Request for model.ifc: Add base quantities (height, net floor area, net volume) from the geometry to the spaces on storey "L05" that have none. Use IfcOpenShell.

First a look at what the model holds.

```python
import ifcopenshell
import ifcopenshell.util.element
import ifcopenshell.util.unit

model = ifcopenshell.open("model.ifc")
print(model.schema)
for unit_type in ("LENGTHUNIT", "AREAUNIT", "VOLUMEUNIT"):
    print(unit_type, ifcopenshell.util.unit.calculate_unit_scale(model, unit_type))
storey = next(s for s in model.by_type("IfcBuildingStorey") if s.Name == "L05")
spaces = [e for e in ifcopenshell.util.element.get_decomposition(storey) if e.is_a("IfcSpace")]
for e in sorted(spaces, key=lambda e: e.id()):
    print(e.id(), e.is_a(), e.Name, list(ifcopenshell.util.element.get_psets(e, qtos_only=True)), sep=" | ")
```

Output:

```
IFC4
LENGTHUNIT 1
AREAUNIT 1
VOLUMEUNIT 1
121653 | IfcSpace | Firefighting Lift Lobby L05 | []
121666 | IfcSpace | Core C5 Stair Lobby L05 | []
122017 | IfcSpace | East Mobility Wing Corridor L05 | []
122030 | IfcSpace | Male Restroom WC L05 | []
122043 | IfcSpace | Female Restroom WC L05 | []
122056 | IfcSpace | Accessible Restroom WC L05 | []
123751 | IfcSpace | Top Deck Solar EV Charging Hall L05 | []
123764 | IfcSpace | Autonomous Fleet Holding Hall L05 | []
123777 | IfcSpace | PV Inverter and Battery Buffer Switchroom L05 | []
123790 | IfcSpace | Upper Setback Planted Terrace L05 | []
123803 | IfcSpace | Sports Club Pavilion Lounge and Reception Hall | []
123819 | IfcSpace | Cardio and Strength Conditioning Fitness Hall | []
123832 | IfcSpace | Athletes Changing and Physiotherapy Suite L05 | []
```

```python
import ifcopenshell
import ifcopenshell.api.pset
import ifcopenshell.geom
import ifcopenshell.util.element
import ifcopenshell.util.shape
import ifcopenshell.util.unit

model = ifcopenshell.open("model.ifc")
unit_scale = ifcopenshell.util.unit.calculate_unit_scale(model)
area_scale = ifcopenshell.util.unit.calculate_unit_scale(model, "AREAUNIT")
volume_scale = ifcopenshell.util.unit.calculate_unit_scale(model, "VOLUMEUNIT")
settings = ifcopenshell.geom.settings()

storey = next(s for s in model.by_type("IfcBuildingStorey") if s.Name == "L05")
spaces = [e for e in ifcopenshell.util.element.get_decomposition(storey) if e.is_a("IfcSpace")]

for e in sorted(spaces, key=lambda e: e.id()):
    if ifcopenshell.util.element.get_psets(e, qtos_only=True, should_inherit=False):
        continue
    # Geometry comes back in metres, in the element's own axes.
    shape = ifcopenshell.geom.create_shape(settings, e)
    values = {
        "Height": ifcopenshell.util.shape.get_z(shape.geometry) / unit_scale,
        "NetFloorArea": ifcopenshell.util.shape.get_footprint_area(shape.geometry) / area_scale,
        "NetVolume": ifcopenshell.util.shape.get_volume(shape.geometry) / volume_scale,
    }
    qto = ifcopenshell.api.pset.add_qto(model, product=e, name="Qto_SpaceBaseQuantities")
    ifcopenshell.api.pset.edit_qto(model, qto=qto, properties=values)
    print(e.id(), {k: round(v, 3) for k, v in values.items()})

model.write("model_rev.ifc")
```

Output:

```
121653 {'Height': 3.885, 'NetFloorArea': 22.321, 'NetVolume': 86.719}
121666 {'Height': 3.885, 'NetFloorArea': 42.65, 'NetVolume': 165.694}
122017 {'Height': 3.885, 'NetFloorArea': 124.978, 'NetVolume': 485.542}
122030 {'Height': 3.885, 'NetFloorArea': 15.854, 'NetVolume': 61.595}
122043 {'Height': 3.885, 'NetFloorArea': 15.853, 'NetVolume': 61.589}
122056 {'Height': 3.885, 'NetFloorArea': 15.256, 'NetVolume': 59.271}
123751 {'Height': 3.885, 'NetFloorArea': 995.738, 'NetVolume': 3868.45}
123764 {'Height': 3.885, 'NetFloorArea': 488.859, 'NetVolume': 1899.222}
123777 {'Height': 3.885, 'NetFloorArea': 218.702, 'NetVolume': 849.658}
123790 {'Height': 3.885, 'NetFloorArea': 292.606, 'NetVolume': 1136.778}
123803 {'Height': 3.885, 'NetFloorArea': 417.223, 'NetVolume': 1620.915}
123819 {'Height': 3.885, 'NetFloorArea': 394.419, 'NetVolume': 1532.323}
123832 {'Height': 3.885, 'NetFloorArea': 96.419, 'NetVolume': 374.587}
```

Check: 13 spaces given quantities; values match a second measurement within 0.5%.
